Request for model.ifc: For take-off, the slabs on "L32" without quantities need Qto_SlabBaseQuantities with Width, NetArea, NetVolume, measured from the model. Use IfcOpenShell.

First a look at what the model holds.

```python
import ifcopenshell
import ifcopenshell.util.element
import ifcopenshell.util.unit

model = ifcopenshell.open("model.ifc")
print(model.schema)
for unit_type in ("LENGTHUNIT", "AREAUNIT", "VOLUMEUNIT"):
    print(unit_type, ifcopenshell.util.unit.calculate_unit_scale(model, unit_type))
storey = next(s for s in model.by_type("IfcBuildingStorey") if s.Name == "L32")
slabs = [e for e in ifcopenshell.util.element.get_decomposition(storey) if e.is_a("IfcSlab")]
for e in sorted(slabs, key=lambda e: e.id()):
    print(e.id(), e.is_a(), e.Name, list(ifcopenshell.util.element.get_psets(e, qtos_only=True)), sep=" | ")
```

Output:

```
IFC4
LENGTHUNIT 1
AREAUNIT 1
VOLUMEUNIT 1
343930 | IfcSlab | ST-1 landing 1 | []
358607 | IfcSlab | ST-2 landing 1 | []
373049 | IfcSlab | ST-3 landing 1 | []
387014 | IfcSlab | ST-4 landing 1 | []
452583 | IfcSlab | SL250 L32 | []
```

```python
import ifcopenshell
import ifcopenshell.api.pset
import ifcopenshell.geom
import ifcopenshell.util.element
import ifcopenshell.util.shape
import ifcopenshell.util.unit

model = ifcopenshell.open("model.ifc")
unit_scale = ifcopenshell.util.unit.calculate_unit_scale(model)
area_scale = ifcopenshell.util.unit.calculate_unit_scale(model, "AREAUNIT")
volume_scale = ifcopenshell.util.unit.calculate_unit_scale(model, "VOLUMEUNIT")
settings = ifcopenshell.geom.settings()

storey = next(s for s in model.by_type("IfcBuildingStorey") if s.Name == "L32")
slabs = [e for e in ifcopenshell.util.element.get_decomposition(storey) if e.is_a("IfcSlab")]

for e in sorted(slabs, key=lambda e: e.id()):
    if ifcopenshell.util.element.get_psets(e, qtos_only=True, should_inherit=False):
        continue
    # Geometry comes back in metres, in the element's own axes.
    shape = ifcopenshell.geom.create_shape(settings, e)
    values = {
        "Width": ifcopenshell.util.shape.get_z(shape.geometry) / unit_scale,
        "NetArea": ifcopenshell.util.shape.get_footprint_area(shape.geometry) / area_scale,
        "NetVolume": ifcopenshell.util.shape.get_volume(shape.geometry) / volume_scale,
    }
    qto = ifcopenshell.api.pset.add_qto(model, product=e, name="Qto_SlabBaseQuantities")
    ifcopenshell.api.pset.edit_qto(model, qto=qto, properties=values)
    print(e.id(), {k: round(v, 3) for k, v in values.items()})

model.write("model_v2.ifc")
```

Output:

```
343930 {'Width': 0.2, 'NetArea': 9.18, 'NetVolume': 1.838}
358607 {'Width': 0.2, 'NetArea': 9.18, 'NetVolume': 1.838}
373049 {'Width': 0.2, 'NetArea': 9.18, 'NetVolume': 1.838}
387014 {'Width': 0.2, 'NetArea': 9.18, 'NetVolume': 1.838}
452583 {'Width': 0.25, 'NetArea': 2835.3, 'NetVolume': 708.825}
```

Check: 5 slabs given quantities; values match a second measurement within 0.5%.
